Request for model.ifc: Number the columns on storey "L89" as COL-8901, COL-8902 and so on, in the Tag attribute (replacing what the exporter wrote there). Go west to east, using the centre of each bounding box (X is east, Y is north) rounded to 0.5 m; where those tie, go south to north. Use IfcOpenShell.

First a look at what the model holds.

```python
import ifcopenshell
import ifcopenshell.util.element
import ifcopenshell.util.placement

model = ifcopenshell.open("model.ifc")
print(model.schema)
storey = next(s for s in model.by_type("IfcBuildingStorey") if s.Name == "L89")
columns = [e for e in ifcopenshell.util.element.get_decomposition(storey) if e.is_a("IfcColumn")]
for e in sorted(columns, key=lambda e: e.id()):
    origin = ifcopenshell.util.placement.get_local_placement(e.ObjectPlacement)[:3, 3]
    print(e.id(), e.Tag, e.Name, origin.round(2) + 0.0, sep=" | ")
```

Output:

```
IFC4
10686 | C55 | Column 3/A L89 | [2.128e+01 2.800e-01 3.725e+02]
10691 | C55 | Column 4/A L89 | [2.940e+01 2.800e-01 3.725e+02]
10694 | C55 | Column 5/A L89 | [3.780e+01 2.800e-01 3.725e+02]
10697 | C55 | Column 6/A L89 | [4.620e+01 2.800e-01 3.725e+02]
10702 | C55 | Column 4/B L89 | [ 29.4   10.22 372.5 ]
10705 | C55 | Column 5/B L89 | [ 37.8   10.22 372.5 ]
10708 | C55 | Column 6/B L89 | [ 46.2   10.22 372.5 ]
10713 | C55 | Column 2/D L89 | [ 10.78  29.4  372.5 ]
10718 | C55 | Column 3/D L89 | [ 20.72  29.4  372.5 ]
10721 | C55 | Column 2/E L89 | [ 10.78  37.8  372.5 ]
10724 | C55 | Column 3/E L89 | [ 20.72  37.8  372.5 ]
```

```python
import ifcopenshell
import ifcopenshell.geom
import ifcopenshell.util.element
import ifcopenshell.util.shape

model = ifcopenshell.open("model.ifc")
settings = ifcopenshell.geom.settings()
settings.set("use-world-coords", True)


def centre(element):
    shape = ifcopenshell.geom.create_shape(settings, element)
    return ifcopenshell.util.shape.get_bbox_centroid(shape.geometry)


storey = next(s for s in model.by_type("IfcBuildingStorey") if s.Name == "L89")
columns = [e for e in ifcopenshell.util.element.get_decomposition(storey) if e.is_a("IfcColumn")]

# Insertion points can sit at a corner or the storey origin, so sort by the geometry (in metres).
centres = {e: centre(e) for e in columns}
columns.sort(key=lambda e: (round(centres[e][0] / 0.5), centres[e][1]))

for i, e in enumerate(columns, start=1):
    number = f"COL-89{i:02d}"
    e.Tag = number
    print(e.id(), number)

model.write("model_rev.ifc")
```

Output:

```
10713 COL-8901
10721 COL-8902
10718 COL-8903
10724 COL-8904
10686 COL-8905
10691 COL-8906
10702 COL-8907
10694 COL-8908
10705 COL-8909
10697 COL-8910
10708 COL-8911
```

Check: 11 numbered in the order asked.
